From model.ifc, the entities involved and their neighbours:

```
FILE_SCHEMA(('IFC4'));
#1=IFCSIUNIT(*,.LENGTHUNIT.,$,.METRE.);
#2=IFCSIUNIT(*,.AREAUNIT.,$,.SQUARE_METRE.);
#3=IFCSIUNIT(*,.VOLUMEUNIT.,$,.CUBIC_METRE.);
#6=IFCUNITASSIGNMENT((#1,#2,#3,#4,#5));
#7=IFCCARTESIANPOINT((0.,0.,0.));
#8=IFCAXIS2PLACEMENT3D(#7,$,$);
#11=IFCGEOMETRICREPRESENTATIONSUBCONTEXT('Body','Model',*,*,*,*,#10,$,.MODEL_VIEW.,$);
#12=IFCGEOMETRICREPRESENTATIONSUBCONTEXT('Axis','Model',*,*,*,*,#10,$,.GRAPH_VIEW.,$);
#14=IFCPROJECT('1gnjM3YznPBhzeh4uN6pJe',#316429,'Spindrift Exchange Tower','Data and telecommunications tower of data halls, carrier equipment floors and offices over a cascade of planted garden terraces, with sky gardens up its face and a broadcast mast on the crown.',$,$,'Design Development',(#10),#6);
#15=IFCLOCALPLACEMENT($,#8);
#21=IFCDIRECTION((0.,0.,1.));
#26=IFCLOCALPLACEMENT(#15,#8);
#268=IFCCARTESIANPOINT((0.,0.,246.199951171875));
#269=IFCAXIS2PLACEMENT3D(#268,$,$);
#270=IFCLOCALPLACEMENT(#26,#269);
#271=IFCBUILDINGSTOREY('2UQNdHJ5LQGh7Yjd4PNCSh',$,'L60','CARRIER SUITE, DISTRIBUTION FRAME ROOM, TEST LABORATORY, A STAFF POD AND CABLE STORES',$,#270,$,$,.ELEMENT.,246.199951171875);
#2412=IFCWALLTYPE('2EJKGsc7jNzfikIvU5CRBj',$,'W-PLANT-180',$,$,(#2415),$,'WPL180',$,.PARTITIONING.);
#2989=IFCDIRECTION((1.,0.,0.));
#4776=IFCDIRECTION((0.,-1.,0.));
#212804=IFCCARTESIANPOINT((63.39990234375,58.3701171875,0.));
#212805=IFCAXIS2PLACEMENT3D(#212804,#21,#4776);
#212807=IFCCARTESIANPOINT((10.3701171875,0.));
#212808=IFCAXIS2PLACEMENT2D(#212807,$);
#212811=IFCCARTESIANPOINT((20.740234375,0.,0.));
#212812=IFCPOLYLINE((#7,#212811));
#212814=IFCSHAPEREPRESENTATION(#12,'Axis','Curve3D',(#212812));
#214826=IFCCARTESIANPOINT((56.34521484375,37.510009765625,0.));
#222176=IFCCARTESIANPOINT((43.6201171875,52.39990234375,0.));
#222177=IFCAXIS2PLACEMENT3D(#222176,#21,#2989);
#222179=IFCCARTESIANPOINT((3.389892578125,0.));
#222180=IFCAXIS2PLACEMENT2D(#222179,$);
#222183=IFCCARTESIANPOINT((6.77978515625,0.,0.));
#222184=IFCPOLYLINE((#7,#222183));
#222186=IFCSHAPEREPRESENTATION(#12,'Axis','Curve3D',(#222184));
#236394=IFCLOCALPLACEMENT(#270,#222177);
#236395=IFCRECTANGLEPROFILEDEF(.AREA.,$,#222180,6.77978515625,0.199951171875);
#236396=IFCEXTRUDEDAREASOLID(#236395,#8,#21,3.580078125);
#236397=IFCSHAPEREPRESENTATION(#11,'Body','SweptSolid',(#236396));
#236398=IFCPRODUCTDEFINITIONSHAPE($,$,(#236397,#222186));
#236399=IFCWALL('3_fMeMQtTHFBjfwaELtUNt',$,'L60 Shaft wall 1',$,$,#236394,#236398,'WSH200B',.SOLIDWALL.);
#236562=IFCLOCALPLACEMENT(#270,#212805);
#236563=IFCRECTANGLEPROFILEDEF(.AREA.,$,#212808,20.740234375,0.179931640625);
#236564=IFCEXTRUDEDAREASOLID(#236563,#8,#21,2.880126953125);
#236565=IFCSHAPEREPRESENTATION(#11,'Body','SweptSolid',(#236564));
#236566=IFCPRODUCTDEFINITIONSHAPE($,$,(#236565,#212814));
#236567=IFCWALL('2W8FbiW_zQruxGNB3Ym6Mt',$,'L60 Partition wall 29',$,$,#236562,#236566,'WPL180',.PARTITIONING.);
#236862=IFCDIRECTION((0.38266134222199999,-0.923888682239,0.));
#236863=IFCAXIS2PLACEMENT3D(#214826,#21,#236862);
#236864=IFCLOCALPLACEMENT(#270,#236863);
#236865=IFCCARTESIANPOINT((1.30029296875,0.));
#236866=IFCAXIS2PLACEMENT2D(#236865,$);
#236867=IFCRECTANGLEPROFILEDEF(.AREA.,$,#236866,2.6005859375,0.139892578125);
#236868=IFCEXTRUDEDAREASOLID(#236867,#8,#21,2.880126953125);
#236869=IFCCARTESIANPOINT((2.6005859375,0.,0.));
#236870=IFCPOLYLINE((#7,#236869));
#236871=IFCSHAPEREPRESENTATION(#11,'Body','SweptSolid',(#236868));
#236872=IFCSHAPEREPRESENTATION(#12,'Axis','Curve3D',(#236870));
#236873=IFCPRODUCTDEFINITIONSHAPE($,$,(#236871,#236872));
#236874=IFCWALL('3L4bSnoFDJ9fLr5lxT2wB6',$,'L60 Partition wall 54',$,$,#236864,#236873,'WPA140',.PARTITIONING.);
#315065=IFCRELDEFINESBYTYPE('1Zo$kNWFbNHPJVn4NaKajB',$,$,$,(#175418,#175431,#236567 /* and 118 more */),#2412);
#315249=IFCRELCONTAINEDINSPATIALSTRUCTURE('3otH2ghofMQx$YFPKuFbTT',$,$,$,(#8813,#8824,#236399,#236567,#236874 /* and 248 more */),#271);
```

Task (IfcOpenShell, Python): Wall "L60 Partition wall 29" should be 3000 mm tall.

```python
import ifcopenshell
import ifcopenshell.geom
import ifcopenshell.util.representation
import ifcopenshell.util.shape
import ifcopenshell.util.unit

model = ifcopenshell.open("model.ifc")
unit_scale = ifcopenshell.util.unit.calculate_unit_scale(model)
settings = ifcopenshell.geom.settings()


def volume(element):
    """Net volume in cubic metres, openings subtracted."""
    shape = ifcopenshell.geom.create_shape(settings, element)
    return ifcopenshell.util.shape.get_volume(shape.geometry)


wall = model.by_guid("2W8FbiW_zQruxGNB3Ym6Mt")
before = volume(wall)

body = ifcopenshell.util.representation.get_representation(wall, "Model", "Body")
solid = body.Items[0]
old_height = solid.Depth
solid.Depth = 3 / unit_scale
after = volume(wall)

print(f"height {old_height:g} -> {solid.Depth:g}, volume {before:.3f} -> {after:.3f} m3")

model.write("model_rev.ifc")
```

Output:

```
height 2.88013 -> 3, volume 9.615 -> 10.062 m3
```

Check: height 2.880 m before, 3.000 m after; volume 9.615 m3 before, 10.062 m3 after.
